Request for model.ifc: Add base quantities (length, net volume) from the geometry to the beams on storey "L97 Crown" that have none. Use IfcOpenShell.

First a look at what the model holds.

```python
import ifcopenshell
import ifcopenshell.util.element
import ifcopenshell.util.unit

model = ifcopenshell.open("model.ifc")
print(model.schema)
for unit_type in ("LENGTHUNIT", "AREAUNIT", "VOLUMEUNIT"):
    print(unit_type, ifcopenshell.util.unit.calculate_unit_scale(model, unit_type))
storey = next(s for s in model.by_type("IfcBuildingStorey") if s.Name == "L97 Crown")
beams = [e for e in ifcopenshell.util.element.get_decomposition(storey) if e.is_a("IfcBeam")]
for e in sorted(beams, key=lambda e: e.id()):
    print(e.id(), e.is_a(), e.Name, list(ifcopenshell.util.element.get_psets(e, qtos_only=True)), sep=" | ")
```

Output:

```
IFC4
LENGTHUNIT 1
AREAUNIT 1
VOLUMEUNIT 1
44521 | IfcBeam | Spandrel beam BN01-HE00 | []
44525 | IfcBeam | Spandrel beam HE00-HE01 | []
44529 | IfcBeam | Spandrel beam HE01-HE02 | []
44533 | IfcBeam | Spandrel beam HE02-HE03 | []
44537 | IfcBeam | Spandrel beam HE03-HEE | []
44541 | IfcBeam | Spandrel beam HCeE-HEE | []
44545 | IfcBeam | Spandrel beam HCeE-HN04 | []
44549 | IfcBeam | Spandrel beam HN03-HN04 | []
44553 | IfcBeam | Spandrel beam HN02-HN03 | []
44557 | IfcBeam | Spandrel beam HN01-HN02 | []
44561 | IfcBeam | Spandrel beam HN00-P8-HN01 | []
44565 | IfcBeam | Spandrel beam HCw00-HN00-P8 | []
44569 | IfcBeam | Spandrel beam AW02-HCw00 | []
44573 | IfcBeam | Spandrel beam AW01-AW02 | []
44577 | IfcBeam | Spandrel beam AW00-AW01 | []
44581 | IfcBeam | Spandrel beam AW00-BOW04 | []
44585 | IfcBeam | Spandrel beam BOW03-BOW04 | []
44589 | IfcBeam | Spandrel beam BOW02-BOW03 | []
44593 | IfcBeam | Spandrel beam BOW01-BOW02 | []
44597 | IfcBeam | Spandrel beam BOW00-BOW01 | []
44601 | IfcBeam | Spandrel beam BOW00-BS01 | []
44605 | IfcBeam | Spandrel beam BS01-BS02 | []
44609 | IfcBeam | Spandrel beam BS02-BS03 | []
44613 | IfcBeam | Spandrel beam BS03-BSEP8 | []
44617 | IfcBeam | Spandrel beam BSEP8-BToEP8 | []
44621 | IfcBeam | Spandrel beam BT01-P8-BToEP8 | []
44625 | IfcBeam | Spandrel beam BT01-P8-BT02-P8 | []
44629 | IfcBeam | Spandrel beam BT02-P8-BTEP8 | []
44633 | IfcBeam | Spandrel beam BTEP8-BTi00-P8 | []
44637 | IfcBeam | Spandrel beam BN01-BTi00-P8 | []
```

```python
import ifcopenshell
import ifcopenshell.api.pset
import ifcopenshell.geom
import ifcopenshell.util.element
import ifcopenshell.util.shape
import ifcopenshell.util.unit

model = ifcopenshell.open("model.ifc")
unit_scale = ifcopenshell.util.unit.calculate_unit_scale(model)
volume_scale = ifcopenshell.util.unit.calculate_unit_scale(model, "VOLUMEUNIT")
settings = ifcopenshell.geom.settings()

storey = next(s for s in model.by_type("IfcBuildingStorey") if s.Name == "L97 Crown")
beams = [e for e in ifcopenshell.util.element.get_decomposition(storey) if e.is_a("IfcBeam")]

for e in sorted(beams, key=lambda e: e.id()):
    if ifcopenshell.util.element.get_psets(e, qtos_only=True, should_inherit=False):
        continue
    # Geometry comes back in metres, in the element's own axes.
    shape = ifcopenshell.geom.create_shape(settings, e)
    values = {
        "Length": ifcopenshell.util.shape.get_max_xyz(shape.geometry) / unit_scale,
        "NetVolume": ifcopenshell.util.shape.get_volume(shape.geometry) / volume_scale,
    }
    qto = ifcopenshell.api.pset.add_qto(model, product=e, name="Qto_BeamBaseQuantities")
    ifcopenshell.api.pset.edit_qto(model, qto=qto, properties=values)
    print(e.id(), {k: round(v, 3) for k, v in values.items()})

model.write("model_v2.ifc")
```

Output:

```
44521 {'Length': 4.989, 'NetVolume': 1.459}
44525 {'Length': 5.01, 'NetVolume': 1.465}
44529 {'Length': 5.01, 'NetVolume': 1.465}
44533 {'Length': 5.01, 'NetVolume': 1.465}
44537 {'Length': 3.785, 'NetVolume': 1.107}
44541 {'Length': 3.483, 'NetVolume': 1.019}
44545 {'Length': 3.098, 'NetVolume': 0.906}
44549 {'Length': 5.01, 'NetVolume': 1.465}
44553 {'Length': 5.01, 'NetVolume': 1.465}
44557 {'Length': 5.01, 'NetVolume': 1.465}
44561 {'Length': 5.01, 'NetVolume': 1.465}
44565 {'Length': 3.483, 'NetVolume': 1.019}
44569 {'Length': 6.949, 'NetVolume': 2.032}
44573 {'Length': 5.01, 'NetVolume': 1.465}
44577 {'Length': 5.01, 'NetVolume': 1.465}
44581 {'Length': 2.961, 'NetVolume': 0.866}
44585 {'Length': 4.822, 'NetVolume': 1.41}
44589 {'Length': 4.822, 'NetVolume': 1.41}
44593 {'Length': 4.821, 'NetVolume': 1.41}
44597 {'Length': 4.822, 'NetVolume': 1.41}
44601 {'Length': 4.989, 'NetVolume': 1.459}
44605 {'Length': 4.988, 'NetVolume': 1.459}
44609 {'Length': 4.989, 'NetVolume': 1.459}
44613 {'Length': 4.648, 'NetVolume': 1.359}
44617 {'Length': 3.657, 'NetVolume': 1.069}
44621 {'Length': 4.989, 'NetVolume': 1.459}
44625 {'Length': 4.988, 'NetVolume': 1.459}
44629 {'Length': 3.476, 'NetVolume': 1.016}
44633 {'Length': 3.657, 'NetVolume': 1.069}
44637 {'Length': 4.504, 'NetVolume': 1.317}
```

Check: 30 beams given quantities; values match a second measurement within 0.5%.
